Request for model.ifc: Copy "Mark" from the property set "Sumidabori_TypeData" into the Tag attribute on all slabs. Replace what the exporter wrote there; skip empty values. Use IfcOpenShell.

First a look at what the model holds.

```python
import ifcopenshell
import ifcopenshell.util.element

model = ifcopenshell.open("model.ifc")
print(model.schema)
slabs = model.by_type("IfcSlab")
print(len(slabs), "slabs")
for e in slabs[:8]:
    source = ifcopenshell.util.element.get_pset(e, "Sumidabori_TypeData", "Mark")
    target = e.Tag
    print(e.id(), repr(source), repr(target), sep=" | ")
```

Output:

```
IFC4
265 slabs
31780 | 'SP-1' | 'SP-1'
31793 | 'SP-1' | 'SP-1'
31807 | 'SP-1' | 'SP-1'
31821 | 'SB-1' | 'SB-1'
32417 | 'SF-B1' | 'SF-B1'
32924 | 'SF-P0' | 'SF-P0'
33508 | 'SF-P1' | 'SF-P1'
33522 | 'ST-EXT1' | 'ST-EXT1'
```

```python
import ifcopenshell
import ifcopenshell.util.element

model = ifcopenshell.open("model.ifc")

count = 0
for e in model.by_type("IfcSlab"):
    value = ifcopenshell.util.element.get_pset(e, "Sumidabori_TypeData", "Mark")
    current = e.Tag
    if not value or not value.strip() or current == value:
        continue
    e.Tag = value
    count += 1

print(count, "slabs updated")

model.write("model-out.ifc")
```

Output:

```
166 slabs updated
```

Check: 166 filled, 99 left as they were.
